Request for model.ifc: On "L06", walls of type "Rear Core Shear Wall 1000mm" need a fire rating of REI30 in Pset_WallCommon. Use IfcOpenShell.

First a look at what the model holds.

```python
import ifcopenshell
import ifcopenshell.util.element

model = ifcopenshell.open("model.ifc")
print(model.schema)
storey = next(s for s in model.by_type("IfcBuildingStorey") if s.Name == "L06")
walls = [e for e in ifcopenshell.util.element.get_decomposition(storey) if e.is_a("IfcWall")]
seen = {}
for e in walls:
    element_type = ifcopenshell.util.element.get_type(e)
    key = (element_type.Name if element_type != e and element_type else None, ifcopenshell.util.element.get_pset(e, "Pset_WallCommon", "FireRating"))
    seen[key] = seen.get(key, 0) + 1
for (name, value), count in sorted(seen.items(), key=str):
    print(count, "x", name, "|", value)
```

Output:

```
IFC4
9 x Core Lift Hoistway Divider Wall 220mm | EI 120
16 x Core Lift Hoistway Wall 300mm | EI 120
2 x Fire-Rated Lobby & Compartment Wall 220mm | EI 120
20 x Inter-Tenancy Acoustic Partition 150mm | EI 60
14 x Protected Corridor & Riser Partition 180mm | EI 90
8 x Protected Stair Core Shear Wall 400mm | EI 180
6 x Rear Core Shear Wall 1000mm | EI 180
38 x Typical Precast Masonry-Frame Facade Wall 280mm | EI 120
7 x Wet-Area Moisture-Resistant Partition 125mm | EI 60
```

```python
import ifcopenshell
import ifcopenshell.api.pset
import ifcopenshell.util.element

model = ifcopenshell.open("model.ifc")

storey = next(s for s in model.by_type("IfcBuildingStorey") if s.Name == "L06")
walls = [e for e in ifcopenshell.util.element.get_decomposition(storey) if e.is_a("IfcWall")]

count = 0
for e in walls:
    element_type = ifcopenshell.util.element.get_type(e)
    if element_type in (None, e) or element_type.Name != "Rear Core Shear Wall 1000mm":
        continue
    # add_pset returns the element's existing set when there is one.
    pset = ifcopenshell.api.pset.add_pset(model, product=e, name="Pset_WallCommon")
    ifcopenshell.api.pset.edit_pset(model, pset=pset, properties={"FireRating": "REI30"})
    count += 1

print(count, "walls updated")

model.write("model_v2.ifc")
```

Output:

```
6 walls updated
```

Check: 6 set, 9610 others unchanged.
